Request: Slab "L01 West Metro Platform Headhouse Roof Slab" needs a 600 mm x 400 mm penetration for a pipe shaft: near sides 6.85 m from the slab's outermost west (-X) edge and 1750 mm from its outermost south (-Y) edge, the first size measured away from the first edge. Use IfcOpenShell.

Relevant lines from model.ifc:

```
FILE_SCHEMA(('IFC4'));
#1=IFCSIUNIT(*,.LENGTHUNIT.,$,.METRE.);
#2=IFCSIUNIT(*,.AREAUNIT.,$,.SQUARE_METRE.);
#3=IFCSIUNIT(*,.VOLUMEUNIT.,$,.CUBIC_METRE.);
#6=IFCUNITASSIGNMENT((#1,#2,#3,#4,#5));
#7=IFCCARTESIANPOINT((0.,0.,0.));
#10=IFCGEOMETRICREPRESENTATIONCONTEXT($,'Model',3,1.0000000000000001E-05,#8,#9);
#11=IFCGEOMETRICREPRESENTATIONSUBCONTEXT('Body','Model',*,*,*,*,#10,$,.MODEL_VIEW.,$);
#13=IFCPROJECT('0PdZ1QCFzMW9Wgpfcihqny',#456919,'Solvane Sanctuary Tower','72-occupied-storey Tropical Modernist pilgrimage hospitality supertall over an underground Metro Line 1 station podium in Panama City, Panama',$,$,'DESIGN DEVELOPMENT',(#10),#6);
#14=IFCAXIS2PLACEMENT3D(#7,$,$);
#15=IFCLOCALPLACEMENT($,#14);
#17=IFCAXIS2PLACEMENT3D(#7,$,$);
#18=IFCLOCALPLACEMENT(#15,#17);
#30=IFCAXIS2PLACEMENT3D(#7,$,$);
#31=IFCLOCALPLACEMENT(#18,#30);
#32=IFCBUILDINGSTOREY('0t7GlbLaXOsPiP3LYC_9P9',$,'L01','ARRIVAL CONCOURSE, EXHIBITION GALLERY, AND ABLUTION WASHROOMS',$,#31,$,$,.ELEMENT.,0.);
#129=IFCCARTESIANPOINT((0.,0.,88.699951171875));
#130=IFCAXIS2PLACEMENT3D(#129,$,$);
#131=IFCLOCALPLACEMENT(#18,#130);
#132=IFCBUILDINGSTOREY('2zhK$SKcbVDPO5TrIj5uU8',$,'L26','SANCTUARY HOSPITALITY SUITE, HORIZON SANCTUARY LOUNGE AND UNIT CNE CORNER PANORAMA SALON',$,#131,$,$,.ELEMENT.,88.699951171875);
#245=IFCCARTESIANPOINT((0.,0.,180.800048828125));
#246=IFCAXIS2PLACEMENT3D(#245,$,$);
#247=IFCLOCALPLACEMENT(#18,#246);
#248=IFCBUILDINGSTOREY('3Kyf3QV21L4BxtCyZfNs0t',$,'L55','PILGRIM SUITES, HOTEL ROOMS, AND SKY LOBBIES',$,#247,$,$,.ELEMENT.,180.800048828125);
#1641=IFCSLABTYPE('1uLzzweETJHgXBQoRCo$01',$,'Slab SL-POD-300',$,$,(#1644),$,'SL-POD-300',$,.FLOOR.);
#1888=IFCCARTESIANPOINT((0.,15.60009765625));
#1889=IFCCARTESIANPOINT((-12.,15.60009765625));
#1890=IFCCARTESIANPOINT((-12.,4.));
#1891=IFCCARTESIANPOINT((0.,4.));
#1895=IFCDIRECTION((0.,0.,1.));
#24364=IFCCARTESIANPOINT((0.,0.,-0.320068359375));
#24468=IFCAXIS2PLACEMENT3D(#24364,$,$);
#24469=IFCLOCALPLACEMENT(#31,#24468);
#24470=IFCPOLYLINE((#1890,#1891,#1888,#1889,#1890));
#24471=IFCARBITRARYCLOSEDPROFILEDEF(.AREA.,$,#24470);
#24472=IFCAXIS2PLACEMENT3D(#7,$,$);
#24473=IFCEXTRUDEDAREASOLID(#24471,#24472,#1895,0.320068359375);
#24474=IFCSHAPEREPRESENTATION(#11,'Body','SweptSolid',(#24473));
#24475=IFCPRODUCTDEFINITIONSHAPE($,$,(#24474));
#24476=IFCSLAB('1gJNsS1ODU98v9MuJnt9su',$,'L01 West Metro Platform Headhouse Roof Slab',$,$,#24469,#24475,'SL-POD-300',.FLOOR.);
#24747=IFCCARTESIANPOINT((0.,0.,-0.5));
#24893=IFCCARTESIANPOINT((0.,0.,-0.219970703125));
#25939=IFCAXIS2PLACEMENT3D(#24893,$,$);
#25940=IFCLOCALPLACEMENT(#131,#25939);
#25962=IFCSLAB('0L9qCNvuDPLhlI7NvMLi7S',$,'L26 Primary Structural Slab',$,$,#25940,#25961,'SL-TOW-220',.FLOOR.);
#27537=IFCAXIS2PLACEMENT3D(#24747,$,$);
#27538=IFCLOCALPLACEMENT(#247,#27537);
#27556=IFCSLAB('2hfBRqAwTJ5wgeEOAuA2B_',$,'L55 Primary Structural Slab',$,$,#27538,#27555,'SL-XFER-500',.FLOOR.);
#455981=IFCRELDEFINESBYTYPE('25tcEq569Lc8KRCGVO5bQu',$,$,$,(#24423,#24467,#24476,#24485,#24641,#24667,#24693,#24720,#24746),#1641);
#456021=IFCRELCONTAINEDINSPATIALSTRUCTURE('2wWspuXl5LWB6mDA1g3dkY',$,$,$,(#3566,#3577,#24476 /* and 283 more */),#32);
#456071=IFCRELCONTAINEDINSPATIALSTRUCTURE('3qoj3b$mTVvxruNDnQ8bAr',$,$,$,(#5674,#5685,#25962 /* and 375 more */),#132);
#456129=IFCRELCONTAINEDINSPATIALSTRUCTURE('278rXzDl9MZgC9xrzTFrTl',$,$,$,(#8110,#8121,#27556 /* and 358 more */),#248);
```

```python
import numpy as np
import ifcopenshell
import ifcopenshell.api.feature
import ifcopenshell.api.geometry
import ifcopenshell.api.root
import ifcopenshell.geom
import ifcopenshell.util.placement
import ifcopenshell.util.representation
import ifcopenshell.util.shape
import ifcopenshell.util.unit

model = ifcopenshell.open("model.ifc")
unit_scale = ifcopenshell.util.unit.calculate_unit_scale(model)
settings = ifcopenshell.geom.settings()


def volume(element):
    """Net volume in cubic metres, openings subtracted."""
    shape = ifcopenshell.geom.create_shape(settings, element)
    return ifcopenshell.util.shape.get_volume(shape.geometry)


slab = model.by_guid("1gJNsS1ODU98v9MuJnt9su")
before = volume(slab)

# Extent in the slab's own axes, in metres. The edges named are its -X and -Y sides.
slab_shape = ifcopenshell.geom.create_shape(settings, slab)
vertices = ifcopenshell.util.shape.get_vertices(slab_shape.geometry)
x_min, y_min, bottom = vertices.min(axis=0)
top = vertices[:, 2].max()

opening = ifcopenshell.api.root.create_entity(model, ifc_class="IfcOpeningElement", name="Pipe shaft opening", predefined_type="OPENING")
context = ifcopenshell.util.representation.get_context(model, "Model", "Body", "MODEL_VIEW")
width, depth = 0.6, 0.4
outline = [(0.0, 0.0), (width, 0.0), (width, depth), (0.0, depth), (0.0, 0.0)]
# Overshoot both faces by 50 mm so the cut is clean.
shape = ifcopenshell.api.geometry.add_slab_representation(
    model, context=context, depth=top - bottom + 0.1, polyline=outline
)
ifcopenshell.api.geometry.assign_representation(model, product=opening, representation=shape)

matrix = ifcopenshell.util.placement.get_local_placement(slab.ObjectPlacement)
matrix[:, 3] = matrix @ np.append(np.array([x_min + 6.85, y_min + 1.75, bottom - 0.05]) / unit_scale, 1.0)
ifcopenshell.api.geometry.edit_object_placement(model, product=opening, matrix=matrix, is_si=False)
ifcopenshell.api.feature.add_feature(model, feature=opening, element=slab)

after = volume(slab)

print(f"slab volume {before:.3f} -> {after:.3f} m3")

model.write("model_updated.ifc")
```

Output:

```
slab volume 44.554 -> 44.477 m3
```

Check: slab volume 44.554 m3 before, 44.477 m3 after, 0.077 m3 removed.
